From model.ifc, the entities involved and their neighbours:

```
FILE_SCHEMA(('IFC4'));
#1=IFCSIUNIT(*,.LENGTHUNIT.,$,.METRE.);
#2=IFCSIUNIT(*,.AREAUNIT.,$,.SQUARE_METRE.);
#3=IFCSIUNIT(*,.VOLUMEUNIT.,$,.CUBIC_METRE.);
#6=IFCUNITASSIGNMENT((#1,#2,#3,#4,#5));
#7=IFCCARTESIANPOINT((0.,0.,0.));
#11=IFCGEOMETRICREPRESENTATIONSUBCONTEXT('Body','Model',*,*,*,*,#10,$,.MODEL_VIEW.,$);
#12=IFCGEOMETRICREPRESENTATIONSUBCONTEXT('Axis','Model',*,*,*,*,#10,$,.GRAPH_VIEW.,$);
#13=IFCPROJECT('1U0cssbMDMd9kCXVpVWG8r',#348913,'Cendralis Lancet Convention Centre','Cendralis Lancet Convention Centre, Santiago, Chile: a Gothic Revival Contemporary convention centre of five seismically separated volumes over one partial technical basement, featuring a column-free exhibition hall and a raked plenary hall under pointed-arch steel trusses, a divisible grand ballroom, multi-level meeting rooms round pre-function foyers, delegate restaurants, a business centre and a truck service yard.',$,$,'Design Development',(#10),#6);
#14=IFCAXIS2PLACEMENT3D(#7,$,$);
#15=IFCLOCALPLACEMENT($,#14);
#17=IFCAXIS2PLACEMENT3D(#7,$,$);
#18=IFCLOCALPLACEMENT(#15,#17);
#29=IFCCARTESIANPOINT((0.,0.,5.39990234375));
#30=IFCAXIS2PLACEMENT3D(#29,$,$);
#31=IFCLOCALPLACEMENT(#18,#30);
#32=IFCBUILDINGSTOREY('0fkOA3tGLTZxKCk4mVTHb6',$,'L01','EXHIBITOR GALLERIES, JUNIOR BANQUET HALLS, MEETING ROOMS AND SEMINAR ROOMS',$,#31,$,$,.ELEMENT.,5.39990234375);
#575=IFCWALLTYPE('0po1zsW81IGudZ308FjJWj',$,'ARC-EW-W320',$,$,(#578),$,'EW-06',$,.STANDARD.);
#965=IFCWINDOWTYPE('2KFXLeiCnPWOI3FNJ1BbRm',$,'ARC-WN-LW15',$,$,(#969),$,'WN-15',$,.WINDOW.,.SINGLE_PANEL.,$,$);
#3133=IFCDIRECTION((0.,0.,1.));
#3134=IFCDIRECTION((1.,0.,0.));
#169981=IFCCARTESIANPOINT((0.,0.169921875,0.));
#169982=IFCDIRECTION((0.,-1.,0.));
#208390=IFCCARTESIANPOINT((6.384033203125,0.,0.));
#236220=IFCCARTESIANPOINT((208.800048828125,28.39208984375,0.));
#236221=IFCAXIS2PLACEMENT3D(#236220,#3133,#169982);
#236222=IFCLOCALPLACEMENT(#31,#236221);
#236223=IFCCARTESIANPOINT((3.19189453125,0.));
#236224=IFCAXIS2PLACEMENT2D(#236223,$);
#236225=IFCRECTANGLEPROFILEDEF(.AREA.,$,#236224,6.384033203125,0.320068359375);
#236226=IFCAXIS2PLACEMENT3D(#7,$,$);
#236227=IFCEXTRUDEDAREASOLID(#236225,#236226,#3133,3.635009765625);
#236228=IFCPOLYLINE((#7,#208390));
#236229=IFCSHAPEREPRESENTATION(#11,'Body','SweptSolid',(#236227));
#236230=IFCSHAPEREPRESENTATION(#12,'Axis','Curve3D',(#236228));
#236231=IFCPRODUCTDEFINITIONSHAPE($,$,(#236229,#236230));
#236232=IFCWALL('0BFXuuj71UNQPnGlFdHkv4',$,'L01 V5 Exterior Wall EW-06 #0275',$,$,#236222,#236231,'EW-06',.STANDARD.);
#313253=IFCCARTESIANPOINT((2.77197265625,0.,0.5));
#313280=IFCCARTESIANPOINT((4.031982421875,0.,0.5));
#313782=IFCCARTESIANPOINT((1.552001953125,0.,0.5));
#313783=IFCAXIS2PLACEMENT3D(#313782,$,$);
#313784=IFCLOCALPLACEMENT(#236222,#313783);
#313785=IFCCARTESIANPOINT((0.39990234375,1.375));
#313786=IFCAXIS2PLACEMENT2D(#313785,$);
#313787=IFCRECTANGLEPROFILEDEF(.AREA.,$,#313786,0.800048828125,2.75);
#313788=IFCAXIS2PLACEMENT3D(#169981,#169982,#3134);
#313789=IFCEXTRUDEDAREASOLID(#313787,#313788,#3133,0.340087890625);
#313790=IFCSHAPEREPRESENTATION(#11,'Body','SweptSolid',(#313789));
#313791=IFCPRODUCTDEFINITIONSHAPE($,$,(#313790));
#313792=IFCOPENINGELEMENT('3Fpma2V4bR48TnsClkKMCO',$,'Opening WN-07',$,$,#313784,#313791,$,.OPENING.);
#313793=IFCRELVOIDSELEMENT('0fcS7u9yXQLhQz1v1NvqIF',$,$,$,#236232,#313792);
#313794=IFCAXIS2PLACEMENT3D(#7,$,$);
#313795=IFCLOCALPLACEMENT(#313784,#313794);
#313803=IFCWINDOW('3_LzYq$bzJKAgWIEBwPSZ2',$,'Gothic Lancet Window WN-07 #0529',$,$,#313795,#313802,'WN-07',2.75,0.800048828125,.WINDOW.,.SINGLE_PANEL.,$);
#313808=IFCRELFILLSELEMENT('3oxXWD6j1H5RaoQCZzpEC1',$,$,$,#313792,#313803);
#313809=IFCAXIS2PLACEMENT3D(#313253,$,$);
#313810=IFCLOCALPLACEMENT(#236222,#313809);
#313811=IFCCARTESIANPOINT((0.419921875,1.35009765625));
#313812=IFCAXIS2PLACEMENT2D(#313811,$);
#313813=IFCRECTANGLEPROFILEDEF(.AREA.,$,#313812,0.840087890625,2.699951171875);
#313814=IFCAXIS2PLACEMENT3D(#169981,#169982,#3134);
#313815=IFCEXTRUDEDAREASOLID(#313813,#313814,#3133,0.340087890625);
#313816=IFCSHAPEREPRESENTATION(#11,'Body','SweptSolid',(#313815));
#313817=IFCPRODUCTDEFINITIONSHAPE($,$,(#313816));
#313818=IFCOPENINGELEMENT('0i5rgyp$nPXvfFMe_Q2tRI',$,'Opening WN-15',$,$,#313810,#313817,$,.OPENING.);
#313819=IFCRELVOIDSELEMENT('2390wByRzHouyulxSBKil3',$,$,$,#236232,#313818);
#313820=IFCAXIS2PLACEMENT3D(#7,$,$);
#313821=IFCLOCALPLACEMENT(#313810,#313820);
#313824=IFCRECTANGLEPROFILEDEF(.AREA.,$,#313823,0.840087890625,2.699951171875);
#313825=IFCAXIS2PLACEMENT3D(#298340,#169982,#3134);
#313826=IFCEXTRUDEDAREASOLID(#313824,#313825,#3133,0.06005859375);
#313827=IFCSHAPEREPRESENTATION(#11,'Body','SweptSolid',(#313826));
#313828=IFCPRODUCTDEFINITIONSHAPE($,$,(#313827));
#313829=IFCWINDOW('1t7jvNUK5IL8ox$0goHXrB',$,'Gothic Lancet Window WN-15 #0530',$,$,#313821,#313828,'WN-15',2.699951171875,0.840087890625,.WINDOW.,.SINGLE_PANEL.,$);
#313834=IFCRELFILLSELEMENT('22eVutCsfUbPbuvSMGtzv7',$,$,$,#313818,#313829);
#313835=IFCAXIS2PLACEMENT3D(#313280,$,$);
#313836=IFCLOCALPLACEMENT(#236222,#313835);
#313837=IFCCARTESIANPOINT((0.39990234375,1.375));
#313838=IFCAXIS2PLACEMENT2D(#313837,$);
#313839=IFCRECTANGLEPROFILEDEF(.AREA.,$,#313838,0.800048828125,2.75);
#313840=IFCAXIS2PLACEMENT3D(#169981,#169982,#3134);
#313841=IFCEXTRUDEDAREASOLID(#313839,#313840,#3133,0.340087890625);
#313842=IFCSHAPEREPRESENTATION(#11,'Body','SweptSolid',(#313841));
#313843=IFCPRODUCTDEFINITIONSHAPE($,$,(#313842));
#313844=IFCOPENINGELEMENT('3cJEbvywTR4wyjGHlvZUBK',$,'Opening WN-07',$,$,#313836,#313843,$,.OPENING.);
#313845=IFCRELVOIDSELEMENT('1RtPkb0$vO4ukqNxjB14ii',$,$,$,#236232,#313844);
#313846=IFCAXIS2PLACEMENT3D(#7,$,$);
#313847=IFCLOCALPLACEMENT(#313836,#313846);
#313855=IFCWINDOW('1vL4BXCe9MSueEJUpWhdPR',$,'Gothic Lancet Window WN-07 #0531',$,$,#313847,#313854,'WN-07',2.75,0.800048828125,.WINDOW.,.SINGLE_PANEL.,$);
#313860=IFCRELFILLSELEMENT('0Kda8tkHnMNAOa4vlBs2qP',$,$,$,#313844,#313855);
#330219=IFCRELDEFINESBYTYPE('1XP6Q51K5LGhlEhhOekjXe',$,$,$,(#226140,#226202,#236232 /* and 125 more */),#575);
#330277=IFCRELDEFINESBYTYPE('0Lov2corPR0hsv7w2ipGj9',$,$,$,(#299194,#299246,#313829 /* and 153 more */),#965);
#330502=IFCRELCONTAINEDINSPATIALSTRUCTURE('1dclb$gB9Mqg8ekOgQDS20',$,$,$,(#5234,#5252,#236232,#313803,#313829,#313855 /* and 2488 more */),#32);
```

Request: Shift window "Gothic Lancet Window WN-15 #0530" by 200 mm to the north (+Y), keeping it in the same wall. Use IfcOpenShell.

```python
import ifcopenshell
import ifcopenshell.api.geometry
import ifcopenshell.util.placement
import ifcopenshell.util.unit

model = ifcopenshell.open("model.ifc")
unit_scale = ifcopenshell.util.unit.calculate_unit_scale(model)

window = model.by_guid("1t7jvNUK5IL8ox$0goHXrB")
opening = window.FillsVoids[0].RelatingOpeningElement
wall = opening.VoidsElements[0].RelatingBuildingElement

wall_matrix = ifcopenshell.util.placement.get_local_placement(wall.ObjectPlacement)
shift = wall_matrix[:3, 0] * -0.2 / unit_scale
before = ifcopenshell.util.placement.get_local_placement(window.ObjectPlacement)[:3, 3].copy()

# The window is placed relative to its opening, so it follows when the opening moves.
matrix = ifcopenshell.util.placement.get_local_placement(opening.ObjectPlacement)
matrix[:3, 3] += shift
ifcopenshell.api.geometry.edit_object_placement(
    model, product=opening, matrix=matrix, is_si=False, should_transform_children=True
)

after = ifcopenshell.util.placement.get_local_placement(window.ObjectPlacement)[:3, 3]
print("window moved by", (after - before).round(3) + 0.0)

model.write("model_rev.ifc")
```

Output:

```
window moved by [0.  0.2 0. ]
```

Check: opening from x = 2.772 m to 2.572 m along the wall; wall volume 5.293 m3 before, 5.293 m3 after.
